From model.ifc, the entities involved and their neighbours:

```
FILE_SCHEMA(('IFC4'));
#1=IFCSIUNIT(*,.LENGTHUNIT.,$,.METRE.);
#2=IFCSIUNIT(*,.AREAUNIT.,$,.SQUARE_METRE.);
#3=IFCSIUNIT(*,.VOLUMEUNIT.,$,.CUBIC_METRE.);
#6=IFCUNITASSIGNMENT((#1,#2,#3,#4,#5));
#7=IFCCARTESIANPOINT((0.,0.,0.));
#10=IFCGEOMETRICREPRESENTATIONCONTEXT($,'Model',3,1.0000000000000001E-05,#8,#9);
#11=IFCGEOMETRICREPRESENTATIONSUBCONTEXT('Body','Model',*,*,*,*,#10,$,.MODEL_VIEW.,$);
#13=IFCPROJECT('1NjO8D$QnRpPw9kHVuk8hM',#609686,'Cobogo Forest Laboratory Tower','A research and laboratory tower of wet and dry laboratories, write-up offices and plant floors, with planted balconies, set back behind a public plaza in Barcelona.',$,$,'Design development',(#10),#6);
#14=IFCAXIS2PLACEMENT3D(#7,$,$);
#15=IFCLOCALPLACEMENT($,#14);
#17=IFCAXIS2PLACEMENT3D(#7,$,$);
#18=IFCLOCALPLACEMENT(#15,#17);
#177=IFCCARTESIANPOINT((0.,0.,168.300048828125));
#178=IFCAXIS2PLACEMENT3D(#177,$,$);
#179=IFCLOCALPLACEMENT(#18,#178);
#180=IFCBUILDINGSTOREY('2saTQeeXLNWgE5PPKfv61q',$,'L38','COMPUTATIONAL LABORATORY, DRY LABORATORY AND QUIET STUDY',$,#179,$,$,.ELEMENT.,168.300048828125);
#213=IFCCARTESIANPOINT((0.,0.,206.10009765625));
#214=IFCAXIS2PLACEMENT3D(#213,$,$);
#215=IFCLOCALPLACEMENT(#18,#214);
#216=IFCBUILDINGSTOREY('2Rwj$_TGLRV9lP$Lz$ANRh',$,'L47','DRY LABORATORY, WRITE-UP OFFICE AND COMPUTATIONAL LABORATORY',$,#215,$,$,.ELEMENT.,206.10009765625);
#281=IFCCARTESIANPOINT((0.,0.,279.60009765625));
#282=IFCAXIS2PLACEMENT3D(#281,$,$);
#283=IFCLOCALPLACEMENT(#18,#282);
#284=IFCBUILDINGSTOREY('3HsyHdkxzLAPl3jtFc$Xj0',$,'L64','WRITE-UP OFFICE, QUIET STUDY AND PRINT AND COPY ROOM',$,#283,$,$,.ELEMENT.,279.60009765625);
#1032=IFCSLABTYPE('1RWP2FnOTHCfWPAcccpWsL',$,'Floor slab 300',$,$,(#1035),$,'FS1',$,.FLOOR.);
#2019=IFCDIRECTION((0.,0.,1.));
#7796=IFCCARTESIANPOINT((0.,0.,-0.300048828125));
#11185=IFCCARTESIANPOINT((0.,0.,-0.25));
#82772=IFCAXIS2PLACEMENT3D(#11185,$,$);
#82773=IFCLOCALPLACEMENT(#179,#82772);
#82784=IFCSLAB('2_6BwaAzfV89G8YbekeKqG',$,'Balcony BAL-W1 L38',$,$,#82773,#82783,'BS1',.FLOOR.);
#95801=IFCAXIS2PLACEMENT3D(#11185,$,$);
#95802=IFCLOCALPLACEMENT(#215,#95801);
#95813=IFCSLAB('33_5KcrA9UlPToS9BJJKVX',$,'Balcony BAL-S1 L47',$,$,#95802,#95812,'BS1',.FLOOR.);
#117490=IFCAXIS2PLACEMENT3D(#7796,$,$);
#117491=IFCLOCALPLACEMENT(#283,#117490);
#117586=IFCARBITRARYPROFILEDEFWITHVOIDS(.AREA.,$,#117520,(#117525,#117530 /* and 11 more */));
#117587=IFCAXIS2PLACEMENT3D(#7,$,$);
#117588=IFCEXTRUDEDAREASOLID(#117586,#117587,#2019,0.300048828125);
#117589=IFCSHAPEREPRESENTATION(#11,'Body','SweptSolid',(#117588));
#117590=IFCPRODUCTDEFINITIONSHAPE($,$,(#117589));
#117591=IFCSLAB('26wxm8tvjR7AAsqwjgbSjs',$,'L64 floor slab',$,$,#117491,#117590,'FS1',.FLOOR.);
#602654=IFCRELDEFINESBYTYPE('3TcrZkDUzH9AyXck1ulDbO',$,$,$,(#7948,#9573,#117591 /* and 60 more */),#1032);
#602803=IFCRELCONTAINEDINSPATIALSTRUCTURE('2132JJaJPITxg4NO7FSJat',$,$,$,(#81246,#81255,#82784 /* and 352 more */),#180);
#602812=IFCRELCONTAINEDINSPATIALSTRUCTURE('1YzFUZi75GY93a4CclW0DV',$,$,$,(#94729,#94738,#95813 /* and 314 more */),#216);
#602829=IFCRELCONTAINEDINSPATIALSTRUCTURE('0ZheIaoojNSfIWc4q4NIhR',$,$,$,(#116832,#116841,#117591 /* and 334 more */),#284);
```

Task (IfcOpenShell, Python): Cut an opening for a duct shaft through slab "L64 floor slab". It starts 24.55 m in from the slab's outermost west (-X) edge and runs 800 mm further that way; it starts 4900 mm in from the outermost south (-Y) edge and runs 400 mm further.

```python
import numpy as np
import ifcopenshell
import ifcopenshell.api.feature
import ifcopenshell.api.geometry
import ifcopenshell.api.root
import ifcopenshell.geom
import ifcopenshell.util.placement
import ifcopenshell.util.representation
import ifcopenshell.util.shape
import ifcopenshell.util.unit

model = ifcopenshell.open("model.ifc")
unit_scale = ifcopenshell.util.unit.calculate_unit_scale(model)
settings = ifcopenshell.geom.settings()


def volume(element):
    """Net volume in cubic metres, openings subtracted."""
    shape = ifcopenshell.geom.create_shape(settings, element)
    return ifcopenshell.util.shape.get_volume(shape.geometry)


slab = model.by_guid("26wxm8tvjR7AAsqwjgbSjs")
before = volume(slab)

# Extent in the slab's own axes, in metres. The edges named are its -X and -Y sides.
slab_shape = ifcopenshell.geom.create_shape(settings, slab)
vertices = ifcopenshell.util.shape.get_vertices(slab_shape.geometry)
x_min, y_min, bottom = vertices.min(axis=0)
top = vertices[:, 2].max()

opening = ifcopenshell.api.root.create_entity(model, ifc_class="IfcOpeningElement", name="Duct shaft opening", predefined_type="OPENING")
context = ifcopenshell.util.representation.get_context(model, "Model", "Body", "MODEL_VIEW")
width, depth = 0.8, 0.4
outline = [(0.0, 0.0), (width, 0.0), (width, depth), (0.0, depth), (0.0, 0.0)]
# Overshoot both faces by 50 mm so the cut is clean.
shape = ifcopenshell.api.geometry.add_slab_representation(
    model, context=context, depth=top - bottom + 0.1, polyline=outline
)
ifcopenshell.api.geometry.assign_representation(model, product=opening, representation=shape)

matrix = ifcopenshell.util.placement.get_local_placement(slab.ObjectPlacement)
matrix[:, 3] = matrix @ np.append(np.array([x_min + 24.55, y_min + 4.9, bottom - 0.05]) / unit_scale, 1.0)
ifcopenshell.api.geometry.edit_object_placement(model, product=opening, matrix=matrix, is_si=False)
ifcopenshell.api.feature.add_feature(model, feature=opening, element=slab)

after = volume(slab)

print(f"slab volume {before:.3f} -> {after:.3f} m3")

model.write("model_edited.ifc")
```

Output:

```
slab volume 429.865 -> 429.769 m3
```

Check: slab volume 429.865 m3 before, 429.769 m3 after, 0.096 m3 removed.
